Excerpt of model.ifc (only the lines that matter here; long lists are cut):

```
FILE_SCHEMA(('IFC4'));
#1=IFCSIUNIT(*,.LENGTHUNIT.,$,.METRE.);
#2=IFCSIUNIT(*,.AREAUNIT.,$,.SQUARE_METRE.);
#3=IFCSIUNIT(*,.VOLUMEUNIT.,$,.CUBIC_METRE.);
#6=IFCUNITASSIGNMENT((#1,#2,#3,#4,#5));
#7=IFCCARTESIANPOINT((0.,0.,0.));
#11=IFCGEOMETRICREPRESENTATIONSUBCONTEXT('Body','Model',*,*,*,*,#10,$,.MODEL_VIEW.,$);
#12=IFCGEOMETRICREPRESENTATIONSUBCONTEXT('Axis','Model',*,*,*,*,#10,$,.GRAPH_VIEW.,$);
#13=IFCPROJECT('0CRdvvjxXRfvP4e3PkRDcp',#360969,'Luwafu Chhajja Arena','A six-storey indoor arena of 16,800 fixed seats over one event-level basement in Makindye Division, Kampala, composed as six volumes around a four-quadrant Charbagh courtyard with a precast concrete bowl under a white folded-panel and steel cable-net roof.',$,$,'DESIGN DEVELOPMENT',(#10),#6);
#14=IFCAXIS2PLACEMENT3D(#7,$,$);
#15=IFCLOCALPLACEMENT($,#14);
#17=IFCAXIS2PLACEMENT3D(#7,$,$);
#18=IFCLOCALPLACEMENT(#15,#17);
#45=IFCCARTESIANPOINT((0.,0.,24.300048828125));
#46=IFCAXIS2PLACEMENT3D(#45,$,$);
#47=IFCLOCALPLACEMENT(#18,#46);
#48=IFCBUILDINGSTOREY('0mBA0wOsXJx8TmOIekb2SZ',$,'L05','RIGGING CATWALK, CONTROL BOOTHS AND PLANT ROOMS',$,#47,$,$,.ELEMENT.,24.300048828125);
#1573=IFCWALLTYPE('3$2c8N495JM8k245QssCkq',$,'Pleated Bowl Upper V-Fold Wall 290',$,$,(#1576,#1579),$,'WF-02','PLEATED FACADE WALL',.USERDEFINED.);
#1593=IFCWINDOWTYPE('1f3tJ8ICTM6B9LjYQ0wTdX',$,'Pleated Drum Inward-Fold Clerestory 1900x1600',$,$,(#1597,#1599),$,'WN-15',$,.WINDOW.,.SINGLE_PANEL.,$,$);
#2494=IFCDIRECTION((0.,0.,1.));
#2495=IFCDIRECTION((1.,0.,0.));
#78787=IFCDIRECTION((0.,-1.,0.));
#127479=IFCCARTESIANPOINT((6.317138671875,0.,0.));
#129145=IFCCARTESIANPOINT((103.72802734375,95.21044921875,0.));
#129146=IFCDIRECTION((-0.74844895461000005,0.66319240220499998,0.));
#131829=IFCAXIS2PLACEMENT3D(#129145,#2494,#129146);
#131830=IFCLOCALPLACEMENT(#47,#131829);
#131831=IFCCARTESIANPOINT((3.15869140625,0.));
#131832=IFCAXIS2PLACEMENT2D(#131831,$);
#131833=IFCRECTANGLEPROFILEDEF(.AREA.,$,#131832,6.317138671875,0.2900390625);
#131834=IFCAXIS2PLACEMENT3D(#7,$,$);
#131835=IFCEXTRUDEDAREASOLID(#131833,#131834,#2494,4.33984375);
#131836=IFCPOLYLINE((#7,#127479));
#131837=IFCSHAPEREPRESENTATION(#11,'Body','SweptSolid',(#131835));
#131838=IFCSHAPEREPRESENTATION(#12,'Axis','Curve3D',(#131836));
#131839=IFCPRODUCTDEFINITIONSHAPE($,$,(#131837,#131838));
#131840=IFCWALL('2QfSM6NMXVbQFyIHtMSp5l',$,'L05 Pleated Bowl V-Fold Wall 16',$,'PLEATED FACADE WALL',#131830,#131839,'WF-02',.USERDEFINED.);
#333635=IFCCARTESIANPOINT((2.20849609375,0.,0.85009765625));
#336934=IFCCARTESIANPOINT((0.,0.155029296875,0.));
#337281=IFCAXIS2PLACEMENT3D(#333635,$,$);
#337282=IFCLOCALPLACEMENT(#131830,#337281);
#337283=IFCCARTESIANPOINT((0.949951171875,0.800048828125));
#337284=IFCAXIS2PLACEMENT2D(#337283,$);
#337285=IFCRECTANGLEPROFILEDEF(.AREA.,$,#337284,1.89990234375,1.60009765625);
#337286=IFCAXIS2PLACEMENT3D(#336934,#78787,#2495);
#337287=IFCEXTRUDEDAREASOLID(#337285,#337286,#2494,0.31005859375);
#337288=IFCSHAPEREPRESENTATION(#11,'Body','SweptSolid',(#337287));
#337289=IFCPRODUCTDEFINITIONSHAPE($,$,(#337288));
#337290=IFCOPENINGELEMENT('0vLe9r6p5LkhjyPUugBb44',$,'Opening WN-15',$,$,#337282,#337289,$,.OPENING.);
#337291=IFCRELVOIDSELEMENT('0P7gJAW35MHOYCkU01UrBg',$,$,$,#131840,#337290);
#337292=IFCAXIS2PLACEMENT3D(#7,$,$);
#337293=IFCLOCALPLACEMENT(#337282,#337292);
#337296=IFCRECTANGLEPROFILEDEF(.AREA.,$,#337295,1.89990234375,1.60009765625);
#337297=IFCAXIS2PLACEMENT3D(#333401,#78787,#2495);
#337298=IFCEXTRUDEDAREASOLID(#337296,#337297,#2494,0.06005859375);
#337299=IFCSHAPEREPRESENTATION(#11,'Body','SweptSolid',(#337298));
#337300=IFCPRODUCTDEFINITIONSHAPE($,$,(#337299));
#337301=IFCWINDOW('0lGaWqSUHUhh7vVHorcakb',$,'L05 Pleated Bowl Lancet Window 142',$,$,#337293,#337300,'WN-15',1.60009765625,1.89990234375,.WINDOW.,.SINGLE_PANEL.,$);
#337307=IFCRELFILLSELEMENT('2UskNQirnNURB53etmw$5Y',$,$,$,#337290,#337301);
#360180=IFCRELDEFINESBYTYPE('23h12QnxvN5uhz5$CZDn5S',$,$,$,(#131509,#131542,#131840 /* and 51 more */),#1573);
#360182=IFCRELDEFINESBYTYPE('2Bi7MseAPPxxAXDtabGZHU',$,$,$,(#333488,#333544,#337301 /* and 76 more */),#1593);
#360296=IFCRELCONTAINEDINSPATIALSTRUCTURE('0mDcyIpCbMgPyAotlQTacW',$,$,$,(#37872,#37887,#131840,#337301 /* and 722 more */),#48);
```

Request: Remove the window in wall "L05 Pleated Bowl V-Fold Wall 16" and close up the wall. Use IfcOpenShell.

```python
import ifcopenshell
import ifcopenshell.api.feature
import ifcopenshell.api.root
import ifcopenshell.geom
import ifcopenshell.util.shape

model = ifcopenshell.open("model.ifc")
settings = ifcopenshell.geom.settings()


def volume(element):
    """Net volume in cubic metres, openings subtracted."""
    shape = ifcopenshell.geom.create_shape(settings, element)
    return ifcopenshell.util.shape.get_volume(shape.geometry)


window = model.by_id(337301)
opening = window.FillsVoids[0].RelatingOpeningElement
wall = opening.VoidsElements[0].RelatingBuildingElement
before = volume(wall)

ifcopenshell.api.root.remove_product(model, product=window)
ifcopenshell.api.feature.remove_feature(model, feature=opening)

after = volume(wall)

print(f"wall volume {before:.3f} -> {after:.3f} m3")

model.write("model-out.ifc")
```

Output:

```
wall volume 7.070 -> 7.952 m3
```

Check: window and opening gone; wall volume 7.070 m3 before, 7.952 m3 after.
